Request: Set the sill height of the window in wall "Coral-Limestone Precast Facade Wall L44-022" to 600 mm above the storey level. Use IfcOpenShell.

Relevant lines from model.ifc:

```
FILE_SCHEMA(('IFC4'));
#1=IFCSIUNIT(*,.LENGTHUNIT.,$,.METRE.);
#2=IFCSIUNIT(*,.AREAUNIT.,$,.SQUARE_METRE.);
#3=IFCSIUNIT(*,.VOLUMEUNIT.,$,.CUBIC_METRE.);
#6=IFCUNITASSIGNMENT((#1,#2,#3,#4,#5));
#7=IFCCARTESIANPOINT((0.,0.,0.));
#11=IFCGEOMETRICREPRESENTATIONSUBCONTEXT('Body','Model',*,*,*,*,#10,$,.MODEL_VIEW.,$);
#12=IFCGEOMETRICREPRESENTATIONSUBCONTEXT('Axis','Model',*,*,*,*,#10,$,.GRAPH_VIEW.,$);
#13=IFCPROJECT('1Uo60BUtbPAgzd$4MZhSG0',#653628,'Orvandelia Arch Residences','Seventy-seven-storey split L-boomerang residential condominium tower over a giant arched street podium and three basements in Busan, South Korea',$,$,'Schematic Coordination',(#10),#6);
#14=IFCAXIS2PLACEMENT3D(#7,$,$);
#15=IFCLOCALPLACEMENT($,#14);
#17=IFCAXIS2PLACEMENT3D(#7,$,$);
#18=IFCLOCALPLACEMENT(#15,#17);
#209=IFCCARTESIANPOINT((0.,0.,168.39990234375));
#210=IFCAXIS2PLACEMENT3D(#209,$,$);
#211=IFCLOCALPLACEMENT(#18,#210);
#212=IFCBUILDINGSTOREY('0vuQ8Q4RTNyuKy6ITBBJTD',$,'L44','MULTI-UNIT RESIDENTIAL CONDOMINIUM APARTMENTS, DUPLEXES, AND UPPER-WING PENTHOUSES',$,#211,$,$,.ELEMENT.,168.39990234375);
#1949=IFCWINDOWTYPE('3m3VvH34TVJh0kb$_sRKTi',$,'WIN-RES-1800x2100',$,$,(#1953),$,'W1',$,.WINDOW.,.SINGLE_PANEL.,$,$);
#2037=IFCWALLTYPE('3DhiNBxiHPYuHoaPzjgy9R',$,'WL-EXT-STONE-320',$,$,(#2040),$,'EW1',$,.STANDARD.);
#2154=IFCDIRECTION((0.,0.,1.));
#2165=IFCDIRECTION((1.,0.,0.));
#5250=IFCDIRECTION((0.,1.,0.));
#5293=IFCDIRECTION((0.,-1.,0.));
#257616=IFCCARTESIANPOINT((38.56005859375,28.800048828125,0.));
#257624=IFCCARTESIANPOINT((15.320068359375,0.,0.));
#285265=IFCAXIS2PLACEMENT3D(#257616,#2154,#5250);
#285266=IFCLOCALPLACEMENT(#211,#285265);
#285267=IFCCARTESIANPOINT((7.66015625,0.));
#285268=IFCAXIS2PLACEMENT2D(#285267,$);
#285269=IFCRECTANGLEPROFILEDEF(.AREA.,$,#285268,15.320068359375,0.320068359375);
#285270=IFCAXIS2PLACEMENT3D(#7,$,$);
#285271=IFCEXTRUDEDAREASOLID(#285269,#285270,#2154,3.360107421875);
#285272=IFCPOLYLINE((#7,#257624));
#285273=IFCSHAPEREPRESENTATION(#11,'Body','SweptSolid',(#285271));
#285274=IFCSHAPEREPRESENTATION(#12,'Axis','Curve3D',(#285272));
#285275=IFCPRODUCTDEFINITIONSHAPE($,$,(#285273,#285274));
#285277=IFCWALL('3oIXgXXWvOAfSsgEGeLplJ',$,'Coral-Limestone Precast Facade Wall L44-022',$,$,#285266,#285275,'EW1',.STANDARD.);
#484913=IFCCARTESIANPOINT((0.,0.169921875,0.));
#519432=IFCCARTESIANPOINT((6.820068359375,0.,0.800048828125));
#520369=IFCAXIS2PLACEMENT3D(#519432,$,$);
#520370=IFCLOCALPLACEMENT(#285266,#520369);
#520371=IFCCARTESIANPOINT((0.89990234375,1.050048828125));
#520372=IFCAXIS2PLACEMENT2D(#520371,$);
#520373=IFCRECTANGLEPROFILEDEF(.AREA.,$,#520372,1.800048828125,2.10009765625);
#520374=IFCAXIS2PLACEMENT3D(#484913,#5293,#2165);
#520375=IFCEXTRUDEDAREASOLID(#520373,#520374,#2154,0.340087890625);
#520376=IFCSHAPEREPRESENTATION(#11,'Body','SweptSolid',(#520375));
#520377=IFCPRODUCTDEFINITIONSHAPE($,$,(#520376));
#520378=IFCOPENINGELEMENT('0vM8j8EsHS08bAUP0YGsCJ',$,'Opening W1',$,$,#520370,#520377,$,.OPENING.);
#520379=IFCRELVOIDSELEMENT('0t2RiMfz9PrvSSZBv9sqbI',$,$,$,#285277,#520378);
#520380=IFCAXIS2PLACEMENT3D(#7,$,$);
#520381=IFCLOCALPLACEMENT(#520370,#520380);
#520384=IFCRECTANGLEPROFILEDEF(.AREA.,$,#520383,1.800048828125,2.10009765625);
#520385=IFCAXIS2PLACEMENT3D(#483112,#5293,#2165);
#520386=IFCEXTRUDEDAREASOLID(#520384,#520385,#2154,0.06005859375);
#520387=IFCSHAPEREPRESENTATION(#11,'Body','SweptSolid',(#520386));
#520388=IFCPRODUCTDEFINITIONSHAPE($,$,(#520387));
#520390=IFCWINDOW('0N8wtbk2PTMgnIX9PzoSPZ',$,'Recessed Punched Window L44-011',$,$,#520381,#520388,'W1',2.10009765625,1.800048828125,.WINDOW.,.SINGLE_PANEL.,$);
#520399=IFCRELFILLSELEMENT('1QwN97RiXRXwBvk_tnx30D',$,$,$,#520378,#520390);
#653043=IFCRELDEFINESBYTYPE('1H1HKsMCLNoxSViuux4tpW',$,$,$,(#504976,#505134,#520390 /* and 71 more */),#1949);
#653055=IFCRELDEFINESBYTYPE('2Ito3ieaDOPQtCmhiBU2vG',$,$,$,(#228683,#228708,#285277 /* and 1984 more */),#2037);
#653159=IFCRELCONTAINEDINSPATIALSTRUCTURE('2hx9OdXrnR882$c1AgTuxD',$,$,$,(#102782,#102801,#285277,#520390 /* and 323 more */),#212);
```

```python
import numpy as np
import ifcopenshell
import ifcopenshell.api.geometry
import ifcopenshell.geom
import ifcopenshell.util.element
import ifcopenshell.util.placement
import ifcopenshell.util.shape
import ifcopenshell.util.unit

model = ifcopenshell.open("model.ifc")
unit_scale = ifcopenshell.util.unit.calculate_unit_scale(model)

window = model.by_id(520390)
opening = window.FillsVoids[0].RelatingOpeningElement
storey = ifcopenshell.util.element.get_container(window, ifc_class="IfcBuildingStorey")
level = ifcopenshell.util.placement.get_local_placement(storey.ObjectPlacement)[2, 3]

# The opening's origin need not be at the sill, so measure its lowest point.
shape = ifcopenshell.geom.create_shape(ifcopenshell.geom.settings(), opening)
bottom = ifcopenshell.util.shape.get_shape_bottom_elevation(shape, shape.geometry) / unit_scale
dz = level + 0.6 / unit_scale - bottom

shift = np.array([0.0, 0.0, dz])
# The window is placed relative to its opening, so it follows when the opening moves.
matrix = ifcopenshell.util.placement.get_local_placement(opening.ObjectPlacement)
matrix[:3, 3] += shift
ifcopenshell.api.geometry.edit_object_placement(
    model, product=opening, matrix=matrix, is_si=False, should_transform_children=True
)

print(f"moved by {dz * unit_scale:+.3f} m")

model.write("model_v2.ifc")
```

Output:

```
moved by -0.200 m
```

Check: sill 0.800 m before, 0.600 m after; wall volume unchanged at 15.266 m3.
